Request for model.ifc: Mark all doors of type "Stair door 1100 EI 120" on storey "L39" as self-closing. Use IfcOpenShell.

First a look at what the model holds.

```python
import ifcopenshell
import ifcopenshell.util.element

model = ifcopenshell.open("model.ifc")
print(model.schema)
storey = next(s for s in model.by_type("IfcBuildingStorey") if s.Name == "L39")
doors = [e for e in ifcopenshell.util.element.get_decomposition(storey) if e.is_a("IfcDoor")]
seen = {}
for e in doors:
    element_type = ifcopenshell.util.element.get_type(e)
    key = (element_type.Name if element_type != e and element_type else None, ifcopenshell.util.element.get_pset(e, "Pset_DoorCommon", "SelfClosing"))
    seen[key] = seen.get(key, 0) + 1
for (name, value), count in sorted(seen.items(), key=str):
    print(count, "x", name, "|", value)
```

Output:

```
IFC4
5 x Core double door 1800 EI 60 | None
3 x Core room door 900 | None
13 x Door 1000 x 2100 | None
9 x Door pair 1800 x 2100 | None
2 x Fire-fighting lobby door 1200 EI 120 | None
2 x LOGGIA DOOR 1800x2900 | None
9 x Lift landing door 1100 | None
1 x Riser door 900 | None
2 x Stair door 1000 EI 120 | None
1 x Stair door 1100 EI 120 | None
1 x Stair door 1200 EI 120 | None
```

```python
import ifcopenshell
import ifcopenshell.api.pset
import ifcopenshell.util.element

model = ifcopenshell.open("model.ifc")

storey = next(s for s in model.by_type("IfcBuildingStorey") if s.Name == "L39")
doors = [e for e in ifcopenshell.util.element.get_decomposition(storey) if e.is_a("IfcDoor")]

count = 0
for e in doors:
    element_type = ifcopenshell.util.element.get_type(e)
    if element_type in (None, e) or element_type.Name != "Stair door 1100 EI 120":
        continue
    # add_pset returns the element's existing set when there is one.
    pset = ifcopenshell.api.pset.add_pset(model, product=e, name="Pset_DoorCommon")
    ifcopenshell.api.pset.edit_pset(model, pset=pset, properties={"SelfClosing": True})
    count += 1

print(count, "doors updated")

model.write("model_edited.ifc")
```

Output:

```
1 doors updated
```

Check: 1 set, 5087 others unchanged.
